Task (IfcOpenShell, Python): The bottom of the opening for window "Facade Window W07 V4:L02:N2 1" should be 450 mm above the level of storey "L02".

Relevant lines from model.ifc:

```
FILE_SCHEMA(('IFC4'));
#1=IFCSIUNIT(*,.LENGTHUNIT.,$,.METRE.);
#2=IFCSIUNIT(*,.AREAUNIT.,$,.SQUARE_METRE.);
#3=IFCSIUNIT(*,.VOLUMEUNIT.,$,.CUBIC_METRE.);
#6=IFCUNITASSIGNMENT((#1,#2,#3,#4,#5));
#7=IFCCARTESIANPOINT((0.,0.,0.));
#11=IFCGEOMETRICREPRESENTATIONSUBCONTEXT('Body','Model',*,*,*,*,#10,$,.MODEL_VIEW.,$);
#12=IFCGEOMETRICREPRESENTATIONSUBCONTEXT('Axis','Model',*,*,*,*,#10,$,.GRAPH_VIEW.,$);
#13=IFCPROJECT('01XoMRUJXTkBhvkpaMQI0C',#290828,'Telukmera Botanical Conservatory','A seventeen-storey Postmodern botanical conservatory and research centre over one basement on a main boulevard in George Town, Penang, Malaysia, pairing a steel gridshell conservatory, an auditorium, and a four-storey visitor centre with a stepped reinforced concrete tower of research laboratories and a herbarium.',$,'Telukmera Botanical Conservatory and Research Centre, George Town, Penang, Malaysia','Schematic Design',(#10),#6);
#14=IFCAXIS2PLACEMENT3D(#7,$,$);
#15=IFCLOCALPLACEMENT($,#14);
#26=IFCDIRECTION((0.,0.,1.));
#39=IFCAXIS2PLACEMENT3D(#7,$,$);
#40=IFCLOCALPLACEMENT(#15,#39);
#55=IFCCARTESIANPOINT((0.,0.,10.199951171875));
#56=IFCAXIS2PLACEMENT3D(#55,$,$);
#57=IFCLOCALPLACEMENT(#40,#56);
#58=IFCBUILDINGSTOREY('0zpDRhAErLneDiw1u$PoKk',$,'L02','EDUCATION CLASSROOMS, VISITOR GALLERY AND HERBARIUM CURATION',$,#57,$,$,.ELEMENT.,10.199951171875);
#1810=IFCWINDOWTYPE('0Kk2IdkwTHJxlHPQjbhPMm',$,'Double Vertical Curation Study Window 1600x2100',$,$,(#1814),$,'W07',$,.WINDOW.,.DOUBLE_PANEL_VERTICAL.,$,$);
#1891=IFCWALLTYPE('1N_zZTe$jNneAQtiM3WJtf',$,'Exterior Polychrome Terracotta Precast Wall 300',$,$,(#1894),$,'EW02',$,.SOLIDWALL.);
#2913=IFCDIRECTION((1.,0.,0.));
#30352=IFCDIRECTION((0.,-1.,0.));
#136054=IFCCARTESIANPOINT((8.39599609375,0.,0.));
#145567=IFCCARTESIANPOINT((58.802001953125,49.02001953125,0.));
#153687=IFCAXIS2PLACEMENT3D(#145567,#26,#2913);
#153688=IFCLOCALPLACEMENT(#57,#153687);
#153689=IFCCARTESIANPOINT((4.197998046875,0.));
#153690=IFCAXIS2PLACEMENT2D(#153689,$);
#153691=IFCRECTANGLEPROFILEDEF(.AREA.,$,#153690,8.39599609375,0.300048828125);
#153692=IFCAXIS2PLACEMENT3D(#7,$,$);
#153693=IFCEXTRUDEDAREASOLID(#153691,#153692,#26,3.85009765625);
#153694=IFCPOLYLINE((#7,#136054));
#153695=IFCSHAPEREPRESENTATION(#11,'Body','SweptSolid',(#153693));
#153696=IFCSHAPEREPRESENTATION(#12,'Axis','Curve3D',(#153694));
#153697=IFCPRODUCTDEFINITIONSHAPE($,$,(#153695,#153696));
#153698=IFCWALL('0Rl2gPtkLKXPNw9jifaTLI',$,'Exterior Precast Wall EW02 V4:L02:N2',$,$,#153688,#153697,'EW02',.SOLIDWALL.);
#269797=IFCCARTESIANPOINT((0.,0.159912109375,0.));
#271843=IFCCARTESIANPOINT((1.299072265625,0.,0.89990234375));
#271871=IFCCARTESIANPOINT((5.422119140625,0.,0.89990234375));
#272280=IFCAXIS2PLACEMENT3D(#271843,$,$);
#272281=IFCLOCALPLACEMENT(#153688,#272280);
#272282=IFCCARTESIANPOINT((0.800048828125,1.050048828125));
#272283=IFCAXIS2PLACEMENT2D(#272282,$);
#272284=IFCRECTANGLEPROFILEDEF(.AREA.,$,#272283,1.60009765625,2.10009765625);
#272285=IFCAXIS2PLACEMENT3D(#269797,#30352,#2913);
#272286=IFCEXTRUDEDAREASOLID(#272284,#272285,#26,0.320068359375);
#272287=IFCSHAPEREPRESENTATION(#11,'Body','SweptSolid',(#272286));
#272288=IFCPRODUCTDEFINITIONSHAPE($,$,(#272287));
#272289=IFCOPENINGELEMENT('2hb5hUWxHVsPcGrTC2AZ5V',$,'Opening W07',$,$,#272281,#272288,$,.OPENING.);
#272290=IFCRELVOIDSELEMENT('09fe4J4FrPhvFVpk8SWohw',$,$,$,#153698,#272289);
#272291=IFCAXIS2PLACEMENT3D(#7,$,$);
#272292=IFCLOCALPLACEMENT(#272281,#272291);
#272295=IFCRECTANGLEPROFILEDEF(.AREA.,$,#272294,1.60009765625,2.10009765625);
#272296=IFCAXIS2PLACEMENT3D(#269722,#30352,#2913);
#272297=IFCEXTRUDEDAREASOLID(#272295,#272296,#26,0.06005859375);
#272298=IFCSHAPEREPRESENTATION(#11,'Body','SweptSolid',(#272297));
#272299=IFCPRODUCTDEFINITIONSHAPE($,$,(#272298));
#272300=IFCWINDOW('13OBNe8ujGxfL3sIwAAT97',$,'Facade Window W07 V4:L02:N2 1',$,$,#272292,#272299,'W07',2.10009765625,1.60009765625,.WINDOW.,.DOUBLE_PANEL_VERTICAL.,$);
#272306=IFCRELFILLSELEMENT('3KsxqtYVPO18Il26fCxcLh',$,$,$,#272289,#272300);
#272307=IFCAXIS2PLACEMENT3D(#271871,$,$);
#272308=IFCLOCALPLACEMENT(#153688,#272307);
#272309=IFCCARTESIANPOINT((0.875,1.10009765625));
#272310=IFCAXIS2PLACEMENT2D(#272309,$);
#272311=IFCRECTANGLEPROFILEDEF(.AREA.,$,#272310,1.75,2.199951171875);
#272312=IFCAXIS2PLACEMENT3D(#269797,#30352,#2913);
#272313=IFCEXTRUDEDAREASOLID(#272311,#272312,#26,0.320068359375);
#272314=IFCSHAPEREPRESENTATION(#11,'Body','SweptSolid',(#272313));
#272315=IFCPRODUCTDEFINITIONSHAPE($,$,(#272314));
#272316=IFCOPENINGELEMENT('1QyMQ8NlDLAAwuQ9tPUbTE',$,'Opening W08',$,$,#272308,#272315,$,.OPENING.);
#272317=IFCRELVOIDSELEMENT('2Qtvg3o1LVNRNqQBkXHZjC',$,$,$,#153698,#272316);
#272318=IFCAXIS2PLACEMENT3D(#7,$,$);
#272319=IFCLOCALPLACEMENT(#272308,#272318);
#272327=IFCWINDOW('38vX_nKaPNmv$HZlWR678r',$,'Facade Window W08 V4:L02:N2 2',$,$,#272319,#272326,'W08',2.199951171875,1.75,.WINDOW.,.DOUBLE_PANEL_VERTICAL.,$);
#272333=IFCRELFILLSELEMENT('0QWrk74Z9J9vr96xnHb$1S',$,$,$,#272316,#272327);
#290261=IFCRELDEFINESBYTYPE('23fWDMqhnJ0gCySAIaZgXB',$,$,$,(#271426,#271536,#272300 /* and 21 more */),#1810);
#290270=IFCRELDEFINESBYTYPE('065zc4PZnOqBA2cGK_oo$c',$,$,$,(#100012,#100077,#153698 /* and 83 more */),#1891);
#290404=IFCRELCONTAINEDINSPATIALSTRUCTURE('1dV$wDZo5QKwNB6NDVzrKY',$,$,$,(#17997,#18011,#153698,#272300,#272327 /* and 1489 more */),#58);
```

```python
import numpy as np
import ifcopenshell
import ifcopenshell.api.geometry
import ifcopenshell.geom
import ifcopenshell.util.element
import ifcopenshell.util.placement
import ifcopenshell.util.shape
import ifcopenshell.util.unit

model = ifcopenshell.open("model.ifc")
unit_scale = ifcopenshell.util.unit.calculate_unit_scale(model)

window = model.by_id(272300)
opening = window.FillsVoids[0].RelatingOpeningElement
storey = ifcopenshell.util.element.get_container(window, ifc_class="IfcBuildingStorey")
level = ifcopenshell.util.placement.get_local_placement(storey.ObjectPlacement)[2, 3]

# The opening's origin need not be at the sill, so measure its lowest point.
shape = ifcopenshell.geom.create_shape(ifcopenshell.geom.settings(), opening)
bottom = ifcopenshell.util.shape.get_shape_bottom_elevation(shape, shape.geometry) / unit_scale
dz = level + 0.45 - bottom

shift = np.array([0.0, 0.0, dz])
# The window is placed relative to its opening, so it follows when the opening moves.
matrix = ifcopenshell.util.placement.get_local_placement(opening.ObjectPlacement)
matrix[:3, 3] += shift
ifcopenshell.api.geometry.edit_object_placement(
    model, product=opening, matrix=matrix, is_si=False, should_transform_children=True
)

print(f"moved by {dz * unit_scale:+.3f} m")

model.write("model_edited.ifc")
```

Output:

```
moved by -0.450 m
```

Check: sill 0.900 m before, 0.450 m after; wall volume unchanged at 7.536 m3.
